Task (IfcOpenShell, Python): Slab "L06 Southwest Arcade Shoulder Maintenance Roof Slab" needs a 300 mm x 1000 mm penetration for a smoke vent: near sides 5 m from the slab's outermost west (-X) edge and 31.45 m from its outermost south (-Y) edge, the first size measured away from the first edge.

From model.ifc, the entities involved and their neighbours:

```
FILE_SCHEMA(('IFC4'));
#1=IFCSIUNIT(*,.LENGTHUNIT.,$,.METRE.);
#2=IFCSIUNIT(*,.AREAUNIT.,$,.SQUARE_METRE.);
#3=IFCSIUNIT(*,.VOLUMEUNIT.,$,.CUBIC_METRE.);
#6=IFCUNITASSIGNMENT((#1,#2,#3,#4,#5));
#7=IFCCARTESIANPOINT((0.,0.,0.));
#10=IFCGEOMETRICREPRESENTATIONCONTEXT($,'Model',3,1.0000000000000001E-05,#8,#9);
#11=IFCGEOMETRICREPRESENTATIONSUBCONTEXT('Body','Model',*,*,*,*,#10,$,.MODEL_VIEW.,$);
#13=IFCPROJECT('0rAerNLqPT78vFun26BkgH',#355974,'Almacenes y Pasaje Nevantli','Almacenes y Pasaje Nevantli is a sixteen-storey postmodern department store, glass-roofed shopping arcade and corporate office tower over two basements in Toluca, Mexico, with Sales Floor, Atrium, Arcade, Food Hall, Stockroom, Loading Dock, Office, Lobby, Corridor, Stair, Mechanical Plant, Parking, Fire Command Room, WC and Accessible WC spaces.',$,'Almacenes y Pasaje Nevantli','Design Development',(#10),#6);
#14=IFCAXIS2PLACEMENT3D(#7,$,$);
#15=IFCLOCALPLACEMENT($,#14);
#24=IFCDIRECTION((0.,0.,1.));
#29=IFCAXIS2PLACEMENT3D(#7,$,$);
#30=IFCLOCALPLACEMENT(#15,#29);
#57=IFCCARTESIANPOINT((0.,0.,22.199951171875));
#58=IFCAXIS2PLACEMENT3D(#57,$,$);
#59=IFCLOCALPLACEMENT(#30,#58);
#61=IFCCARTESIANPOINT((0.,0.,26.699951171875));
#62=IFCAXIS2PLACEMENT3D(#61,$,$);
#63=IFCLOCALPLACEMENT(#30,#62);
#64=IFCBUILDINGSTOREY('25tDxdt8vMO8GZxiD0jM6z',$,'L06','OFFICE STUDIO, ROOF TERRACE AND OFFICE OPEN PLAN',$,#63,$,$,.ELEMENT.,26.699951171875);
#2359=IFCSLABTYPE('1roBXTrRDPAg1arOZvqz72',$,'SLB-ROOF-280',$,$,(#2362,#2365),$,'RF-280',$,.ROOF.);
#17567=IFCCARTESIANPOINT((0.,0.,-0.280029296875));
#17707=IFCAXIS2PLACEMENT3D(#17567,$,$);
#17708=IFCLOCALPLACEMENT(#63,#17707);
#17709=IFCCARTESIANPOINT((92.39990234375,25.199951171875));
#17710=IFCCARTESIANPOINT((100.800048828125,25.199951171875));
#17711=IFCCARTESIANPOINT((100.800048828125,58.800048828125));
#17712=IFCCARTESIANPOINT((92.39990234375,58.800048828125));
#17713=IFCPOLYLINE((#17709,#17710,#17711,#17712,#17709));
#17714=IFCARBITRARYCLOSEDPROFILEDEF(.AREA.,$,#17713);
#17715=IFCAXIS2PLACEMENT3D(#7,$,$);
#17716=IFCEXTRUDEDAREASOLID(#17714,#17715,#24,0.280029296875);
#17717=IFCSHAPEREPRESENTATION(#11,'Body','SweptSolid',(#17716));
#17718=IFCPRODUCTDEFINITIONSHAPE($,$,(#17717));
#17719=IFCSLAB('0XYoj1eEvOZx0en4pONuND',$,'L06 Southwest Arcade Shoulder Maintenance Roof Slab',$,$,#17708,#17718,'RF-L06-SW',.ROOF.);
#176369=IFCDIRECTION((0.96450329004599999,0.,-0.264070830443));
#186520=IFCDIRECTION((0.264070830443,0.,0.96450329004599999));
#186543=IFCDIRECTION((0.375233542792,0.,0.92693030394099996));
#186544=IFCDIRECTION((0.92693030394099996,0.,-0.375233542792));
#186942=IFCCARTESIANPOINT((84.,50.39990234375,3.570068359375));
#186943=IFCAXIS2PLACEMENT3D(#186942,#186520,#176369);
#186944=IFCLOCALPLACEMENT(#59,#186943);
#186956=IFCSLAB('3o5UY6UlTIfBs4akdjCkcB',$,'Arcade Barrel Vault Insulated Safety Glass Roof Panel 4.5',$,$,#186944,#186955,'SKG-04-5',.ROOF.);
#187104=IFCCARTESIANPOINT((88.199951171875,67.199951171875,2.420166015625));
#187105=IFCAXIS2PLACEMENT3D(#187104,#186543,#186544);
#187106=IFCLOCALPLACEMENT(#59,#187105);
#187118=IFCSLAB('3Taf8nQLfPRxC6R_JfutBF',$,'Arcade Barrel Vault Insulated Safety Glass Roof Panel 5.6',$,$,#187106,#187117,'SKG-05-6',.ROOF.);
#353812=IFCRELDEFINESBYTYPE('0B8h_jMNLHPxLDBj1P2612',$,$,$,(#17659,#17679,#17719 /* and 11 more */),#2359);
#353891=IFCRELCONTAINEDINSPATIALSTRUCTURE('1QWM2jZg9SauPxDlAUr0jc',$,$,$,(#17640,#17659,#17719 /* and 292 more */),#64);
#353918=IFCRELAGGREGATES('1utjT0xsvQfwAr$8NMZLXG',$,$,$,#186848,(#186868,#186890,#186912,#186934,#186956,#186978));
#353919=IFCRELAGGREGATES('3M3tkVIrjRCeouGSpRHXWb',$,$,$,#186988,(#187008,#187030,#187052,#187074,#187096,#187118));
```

```python
import numpy as np
import ifcopenshell
import ifcopenshell.api.feature
import ifcopenshell.api.geometry
import ifcopenshell.api.root
import ifcopenshell.geom
import ifcopenshell.util.placement
import ifcopenshell.util.representation
import ifcopenshell.util.shape
import ifcopenshell.util.unit

model = ifcopenshell.open("model.ifc")
unit_scale = ifcopenshell.util.unit.calculate_unit_scale(model)
settings = ifcopenshell.geom.settings()


def volume(element):
    """Net volume in cubic metres, openings subtracted."""
    shape = ifcopenshell.geom.create_shape(settings, element)
    return ifcopenshell.util.shape.get_volume(shape.geometry)


slab = model.by_guid("0XYoj1eEvOZx0en4pONuND")
before = volume(slab)

# Extent in the slab's own axes, in metres. The edges named are its -X and -Y sides.
slab_shape = ifcopenshell.geom.create_shape(settings, slab)
vertices = ifcopenshell.util.shape.get_vertices(slab_shape.geometry)
x_min, y_min, bottom = vertices.min(axis=0)
top = vertices[:, 2].max()

opening = ifcopenshell.api.root.create_entity(model, ifc_class="IfcOpeningElement", name="Smoke vent opening", predefined_type="OPENING")
context = ifcopenshell.util.representation.get_context(model, "Model", "Body", "MODEL_VIEW")
width, depth = 0.3, 1
outline = [(0.0, 0.0), (width, 0.0), (width, depth), (0.0, depth), (0.0, 0.0)]
# Overshoot both faces by 50 mm so the cut is clean.
shape = ifcopenshell.api.geometry.add_slab_representation(
    model, context=context, depth=top - bottom + 0.1, polyline=outline
)
ifcopenshell.api.geometry.assign_representation(model, product=opening, representation=shape)

matrix = ifcopenshell.util.placement.get_local_placement(slab.ObjectPlacement)
matrix[:, 3] = matrix @ np.append(np.array([x_min + 5, y_min + 31.45, bottom - 0.05]) / unit_scale, 1.0)
ifcopenshell.api.geometry.edit_object_placement(model, product=opening, matrix=matrix, is_si=False)
ifcopenshell.api.feature.add_feature(model, feature=opening, element=slab)

after = volume(slab)

print(f"slab volume {before:.3f} -> {after:.3f} m3")

model.write("model_updated.ifc")
```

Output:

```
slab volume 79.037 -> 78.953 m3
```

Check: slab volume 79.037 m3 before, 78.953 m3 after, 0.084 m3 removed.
